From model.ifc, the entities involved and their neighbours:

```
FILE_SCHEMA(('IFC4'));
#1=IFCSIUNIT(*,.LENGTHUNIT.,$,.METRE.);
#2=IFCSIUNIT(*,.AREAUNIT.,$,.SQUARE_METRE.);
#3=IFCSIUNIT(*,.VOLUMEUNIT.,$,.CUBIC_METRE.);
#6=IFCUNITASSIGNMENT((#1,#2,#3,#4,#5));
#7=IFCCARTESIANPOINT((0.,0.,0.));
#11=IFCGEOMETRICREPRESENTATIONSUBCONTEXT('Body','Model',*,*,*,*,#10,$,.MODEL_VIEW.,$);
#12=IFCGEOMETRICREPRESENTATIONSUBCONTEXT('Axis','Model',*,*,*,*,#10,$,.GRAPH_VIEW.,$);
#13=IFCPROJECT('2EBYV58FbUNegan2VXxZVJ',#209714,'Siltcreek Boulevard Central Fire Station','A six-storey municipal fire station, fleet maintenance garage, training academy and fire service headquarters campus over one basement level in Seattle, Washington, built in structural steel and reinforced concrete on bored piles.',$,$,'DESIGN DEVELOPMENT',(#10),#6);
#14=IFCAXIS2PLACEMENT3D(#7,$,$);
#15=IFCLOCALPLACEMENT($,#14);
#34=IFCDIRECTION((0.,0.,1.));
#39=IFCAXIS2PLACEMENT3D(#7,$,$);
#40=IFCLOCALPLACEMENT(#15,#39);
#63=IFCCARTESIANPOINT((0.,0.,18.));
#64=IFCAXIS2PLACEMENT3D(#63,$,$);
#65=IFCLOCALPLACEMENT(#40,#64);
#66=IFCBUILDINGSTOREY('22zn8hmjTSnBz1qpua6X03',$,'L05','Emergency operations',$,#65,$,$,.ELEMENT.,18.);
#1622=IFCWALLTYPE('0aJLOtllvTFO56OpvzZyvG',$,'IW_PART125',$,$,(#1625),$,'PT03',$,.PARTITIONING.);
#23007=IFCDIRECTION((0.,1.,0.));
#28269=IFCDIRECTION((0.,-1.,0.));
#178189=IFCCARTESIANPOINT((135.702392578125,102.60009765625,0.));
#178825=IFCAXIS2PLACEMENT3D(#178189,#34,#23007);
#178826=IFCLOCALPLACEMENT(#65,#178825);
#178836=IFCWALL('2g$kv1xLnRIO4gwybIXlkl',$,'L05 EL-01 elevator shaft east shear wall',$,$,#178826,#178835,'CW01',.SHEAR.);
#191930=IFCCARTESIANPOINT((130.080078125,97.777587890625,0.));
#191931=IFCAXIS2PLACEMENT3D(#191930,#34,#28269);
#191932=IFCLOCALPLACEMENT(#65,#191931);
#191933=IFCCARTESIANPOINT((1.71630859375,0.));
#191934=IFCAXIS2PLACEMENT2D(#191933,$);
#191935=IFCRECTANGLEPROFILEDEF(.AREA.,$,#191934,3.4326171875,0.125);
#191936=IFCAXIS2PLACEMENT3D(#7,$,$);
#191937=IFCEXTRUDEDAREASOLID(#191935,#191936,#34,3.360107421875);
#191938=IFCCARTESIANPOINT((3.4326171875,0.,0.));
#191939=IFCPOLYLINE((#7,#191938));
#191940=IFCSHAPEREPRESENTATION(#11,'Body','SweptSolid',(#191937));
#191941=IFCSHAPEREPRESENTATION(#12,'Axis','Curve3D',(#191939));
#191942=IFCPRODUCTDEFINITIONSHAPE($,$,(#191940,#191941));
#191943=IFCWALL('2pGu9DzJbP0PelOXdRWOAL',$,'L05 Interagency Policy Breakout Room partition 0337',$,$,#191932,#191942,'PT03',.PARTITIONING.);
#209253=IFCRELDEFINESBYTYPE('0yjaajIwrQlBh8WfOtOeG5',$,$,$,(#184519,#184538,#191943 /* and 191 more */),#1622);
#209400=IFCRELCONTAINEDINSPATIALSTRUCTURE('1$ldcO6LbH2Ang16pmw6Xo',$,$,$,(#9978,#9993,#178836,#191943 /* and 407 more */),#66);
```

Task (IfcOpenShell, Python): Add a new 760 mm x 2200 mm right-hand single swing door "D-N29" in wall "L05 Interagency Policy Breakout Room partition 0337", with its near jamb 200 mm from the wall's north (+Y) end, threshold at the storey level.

```python
import numpy as np
import ifcopenshell
import ifcopenshell.api.feature
import ifcopenshell.api.geometry
import ifcopenshell.api.root
import ifcopenshell.api.spatial
import ifcopenshell.geom
import ifcopenshell.util.element
import ifcopenshell.util.placement
import ifcopenshell.util.representation
import ifcopenshell.util.shape
import ifcopenshell.util.unit

model = ifcopenshell.open("model.ifc")
unit_scale = ifcopenshell.util.unit.calculate_unit_scale(model)
settings = ifcopenshell.geom.settings()


def volume(element):
    """Net volume in cubic metres, openings subtracted."""
    shape = ifcopenshell.geom.create_shape(settings, element)
    return ifcopenshell.util.shape.get_volume(shape.geometry)


wall = model.by_id(191943)
storey = ifcopenshell.util.element.get_container(wall, ifc_class="IfcBuildingStorey")
context = ifcopenshell.util.representation.get_context(model, "Model", "Body", "MODEL_VIEW")
before = volume(wall)

width, height, from_end, sill = 0.76, 2.2, 0.2, 0.0  # metres

# The wall runs along its own X axis, and the end named is its -X end.
wall_shape = ifcopenshell.geom.create_shape(settings, wall)
x, y, z = ifcopenshell.util.shape.get_vertices(wall_shape.geometry).T
start = x.min() + from_end
face, thickness = float(y.min()), float(y.max() - y.min())
wall_matrix = ifcopenshell.util.placement.get_local_placement(wall.ObjectPlacement)
level = ifcopenshell.util.placement.get_local_placement(storey.ObjectPlacement)[2, 3]


def in_wall(x, y):
    """Placement at x, y metres in the wall's axes, at sill height."""
    matrix = wall_matrix.copy()
    matrix[:, 3] = wall_matrix @ np.array([x / unit_scale, y / unit_scale, 0.0, 1.0])
    matrix[2, 3] = level + sill / unit_scale
    return matrix


# Opening: a box that overshoots both wall faces by 50 mm.
opening = ifcopenshell.api.root.create_entity(model, ifc_class="IfcOpeningElement", predefined_type="OPENING")
box = ifcopenshell.api.geometry.add_wall_representation(
    model, context=context, length=width, height=height, thickness=thickness + 0.1
)
ifcopenshell.api.geometry.assign_representation(model, product=opening, representation=box)
ifcopenshell.api.geometry.edit_object_placement(model, product=opening, matrix=in_wall(start, face - 0.05), is_si=False)
ifcopenshell.api.feature.add_feature(model, feature=opening, element=wall)

door = ifcopenshell.api.root.create_entity(model, ifc_class="IfcDoor", name="D-N29", predefined_type="DOOR")
door.OverallWidth, door.OverallHeight = width / unit_scale, height / unit_scale
door.OperationType = "SINGLE_SWING_RIGHT"
body = ifcopenshell.api.geometry.add_door_representation(
    model,
    context=context,
    overall_width=door.OverallWidth,
    overall_height=door.OverallHeight,
    operation_type="SINGLE_SWING_RIGHT",
    lining_properties={"LiningDepth": thickness / unit_scale, "ThresholdDepth": thickness / unit_scale},
)
ifcopenshell.api.geometry.assign_representation(model, product=door, representation=body)
ifcopenshell.api.spatial.assign_container(model, products=[door], relating_structure=storey)
ifcopenshell.api.feature.add_filling(model, opening=opening, element=door)

# The lining spans the wall, so the door starts at the wall face.
ifcopenshell.api.geometry.edit_object_placement(model, product=door, matrix=in_wall(start, face), is_si=False)

after = volume(wall)

print(f"wall volume {before:.3f} -> {after:.3f} m3")

model.write("model_updated.ifc")
```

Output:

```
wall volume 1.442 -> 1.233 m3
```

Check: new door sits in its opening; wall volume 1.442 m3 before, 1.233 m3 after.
